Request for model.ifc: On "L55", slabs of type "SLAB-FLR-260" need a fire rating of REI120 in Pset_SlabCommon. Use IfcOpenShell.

First a look at what the model holds.

```python
import ifcopenshell
import ifcopenshell.util.element

model = ifcopenshell.open("model.ifc")
print(model.schema)
storey = next(s for s in model.by_type("IfcBuildingStorey") if s.Name == "L55")
slabs = [e for e in ifcopenshell.util.element.get_decomposition(storey) if e.is_a("IfcSlab")]
seen = {}
for e in slabs:
    element_type = ifcopenshell.util.element.get_type(e)
    key = (element_type.Name if element_type != e and element_type else None, ifcopenshell.util.element.get_pset(e, "Pset_SlabCommon", "FireRating"))
    seen[key] = seen.get(key, 0) + 1
for (name, value), count in sorted(seen.items(), key=str):
    print(count, "x", name, "|", value)
```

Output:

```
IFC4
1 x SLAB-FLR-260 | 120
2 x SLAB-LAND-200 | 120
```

```python
import ifcopenshell
import ifcopenshell.api.pset
import ifcopenshell.util.element

model = ifcopenshell.open("model.ifc")

storey = next(s for s in model.by_type("IfcBuildingStorey") if s.Name == "L55")
slabs = [e for e in ifcopenshell.util.element.get_decomposition(storey) if e.is_a("IfcSlab")]

count = 0
for e in slabs:
    element_type = ifcopenshell.util.element.get_type(e)
    if element_type in (None, e) or element_type.Name != "SLAB-FLR-260":
        continue
    # add_pset returns the element's existing set when there is one.
    pset = ifcopenshell.api.pset.add_pset(model, product=e, name="Pset_SlabCommon")
    ifcopenshell.api.pset.edit_pset(model, pset=pset, properties={"FireRating": "REI120"})
    count += 1

print(count, "slabs updated")

model.write("model_updated.ifc")
```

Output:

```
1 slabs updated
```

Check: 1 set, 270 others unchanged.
